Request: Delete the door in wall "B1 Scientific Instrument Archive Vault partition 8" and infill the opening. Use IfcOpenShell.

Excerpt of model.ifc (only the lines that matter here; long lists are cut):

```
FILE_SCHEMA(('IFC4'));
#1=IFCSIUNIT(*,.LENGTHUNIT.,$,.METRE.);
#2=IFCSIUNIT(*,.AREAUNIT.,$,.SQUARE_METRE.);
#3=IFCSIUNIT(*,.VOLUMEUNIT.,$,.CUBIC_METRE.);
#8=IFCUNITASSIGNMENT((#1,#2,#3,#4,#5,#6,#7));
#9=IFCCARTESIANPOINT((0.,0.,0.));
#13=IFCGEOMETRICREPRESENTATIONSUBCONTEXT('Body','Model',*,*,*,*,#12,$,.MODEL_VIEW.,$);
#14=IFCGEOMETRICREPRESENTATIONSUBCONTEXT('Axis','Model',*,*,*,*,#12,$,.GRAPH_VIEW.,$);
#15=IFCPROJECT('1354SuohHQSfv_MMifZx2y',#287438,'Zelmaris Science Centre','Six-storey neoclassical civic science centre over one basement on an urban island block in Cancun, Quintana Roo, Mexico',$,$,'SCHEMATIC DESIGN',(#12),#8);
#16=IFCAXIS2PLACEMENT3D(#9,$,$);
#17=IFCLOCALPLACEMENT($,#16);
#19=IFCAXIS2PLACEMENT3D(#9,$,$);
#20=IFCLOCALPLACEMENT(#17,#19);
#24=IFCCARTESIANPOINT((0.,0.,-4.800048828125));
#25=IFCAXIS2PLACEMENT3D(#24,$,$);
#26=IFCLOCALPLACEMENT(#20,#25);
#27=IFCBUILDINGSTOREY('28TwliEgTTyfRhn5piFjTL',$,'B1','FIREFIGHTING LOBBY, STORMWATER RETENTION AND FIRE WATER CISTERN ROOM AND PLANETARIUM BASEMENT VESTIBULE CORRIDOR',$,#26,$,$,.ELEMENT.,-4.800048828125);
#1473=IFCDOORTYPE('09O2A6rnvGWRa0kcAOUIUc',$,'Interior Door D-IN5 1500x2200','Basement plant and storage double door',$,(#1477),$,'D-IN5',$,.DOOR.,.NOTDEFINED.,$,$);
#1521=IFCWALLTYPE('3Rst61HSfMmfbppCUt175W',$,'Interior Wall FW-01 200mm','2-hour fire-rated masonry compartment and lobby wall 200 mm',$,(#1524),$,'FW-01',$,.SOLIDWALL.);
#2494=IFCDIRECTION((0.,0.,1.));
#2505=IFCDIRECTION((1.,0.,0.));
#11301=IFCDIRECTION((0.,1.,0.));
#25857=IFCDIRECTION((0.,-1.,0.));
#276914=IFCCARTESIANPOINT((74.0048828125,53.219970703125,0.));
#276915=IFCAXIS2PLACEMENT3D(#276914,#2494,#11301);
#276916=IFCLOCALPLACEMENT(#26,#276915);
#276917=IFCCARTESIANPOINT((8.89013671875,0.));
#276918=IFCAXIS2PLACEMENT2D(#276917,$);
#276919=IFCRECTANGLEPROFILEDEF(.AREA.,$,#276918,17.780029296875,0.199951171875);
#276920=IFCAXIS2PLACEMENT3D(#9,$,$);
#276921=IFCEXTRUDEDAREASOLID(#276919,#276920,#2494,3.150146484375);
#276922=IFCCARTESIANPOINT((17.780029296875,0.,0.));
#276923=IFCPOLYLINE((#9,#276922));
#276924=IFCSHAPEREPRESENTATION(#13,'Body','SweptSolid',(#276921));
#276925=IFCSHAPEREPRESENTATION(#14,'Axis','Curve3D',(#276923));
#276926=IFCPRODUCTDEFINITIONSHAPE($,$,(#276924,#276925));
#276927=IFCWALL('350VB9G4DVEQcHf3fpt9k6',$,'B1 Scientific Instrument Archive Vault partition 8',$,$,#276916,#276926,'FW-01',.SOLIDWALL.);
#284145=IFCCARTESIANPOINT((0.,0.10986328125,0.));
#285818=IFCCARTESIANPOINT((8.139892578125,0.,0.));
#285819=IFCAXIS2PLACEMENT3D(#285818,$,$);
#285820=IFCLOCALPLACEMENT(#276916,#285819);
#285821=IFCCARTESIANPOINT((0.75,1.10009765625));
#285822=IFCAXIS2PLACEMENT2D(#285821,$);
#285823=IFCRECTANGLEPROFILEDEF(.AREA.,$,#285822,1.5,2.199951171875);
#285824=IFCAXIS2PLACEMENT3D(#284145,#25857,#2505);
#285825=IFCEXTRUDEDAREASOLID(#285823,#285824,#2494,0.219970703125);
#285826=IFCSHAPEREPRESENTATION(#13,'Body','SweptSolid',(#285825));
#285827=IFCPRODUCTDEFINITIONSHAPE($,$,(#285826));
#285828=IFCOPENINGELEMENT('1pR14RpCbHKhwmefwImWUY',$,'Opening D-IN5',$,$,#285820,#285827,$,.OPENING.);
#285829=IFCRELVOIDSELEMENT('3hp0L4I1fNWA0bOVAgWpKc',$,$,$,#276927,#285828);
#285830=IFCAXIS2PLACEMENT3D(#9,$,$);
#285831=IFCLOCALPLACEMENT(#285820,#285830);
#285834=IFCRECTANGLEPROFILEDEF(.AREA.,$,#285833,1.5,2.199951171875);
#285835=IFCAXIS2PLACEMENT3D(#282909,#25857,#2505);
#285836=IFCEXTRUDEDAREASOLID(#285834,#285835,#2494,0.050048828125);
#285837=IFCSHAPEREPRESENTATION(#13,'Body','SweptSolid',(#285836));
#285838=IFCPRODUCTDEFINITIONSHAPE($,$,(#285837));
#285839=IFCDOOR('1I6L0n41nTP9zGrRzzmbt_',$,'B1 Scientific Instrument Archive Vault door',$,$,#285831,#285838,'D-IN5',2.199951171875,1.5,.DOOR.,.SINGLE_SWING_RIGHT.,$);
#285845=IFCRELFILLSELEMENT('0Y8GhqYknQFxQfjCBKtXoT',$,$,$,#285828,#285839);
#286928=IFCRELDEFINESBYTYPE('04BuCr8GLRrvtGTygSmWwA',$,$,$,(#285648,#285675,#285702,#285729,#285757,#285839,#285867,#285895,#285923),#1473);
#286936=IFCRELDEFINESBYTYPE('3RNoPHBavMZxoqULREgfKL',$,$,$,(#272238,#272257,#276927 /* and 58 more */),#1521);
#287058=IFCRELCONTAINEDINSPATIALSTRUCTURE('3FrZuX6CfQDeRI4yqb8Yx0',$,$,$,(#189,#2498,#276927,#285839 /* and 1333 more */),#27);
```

```python
import ifcopenshell
import ifcopenshell.api.feature
import ifcopenshell.api.root
import ifcopenshell.geom
import ifcopenshell.util.shape

model = ifcopenshell.open("model.ifc")
settings = ifcopenshell.geom.settings()


def volume(element):
    """Net volume in cubic metres, openings subtracted."""
    shape = ifcopenshell.geom.create_shape(settings, element)
    return ifcopenshell.util.shape.get_volume(shape.geometry)


door = model.by_guid("1I6L0n41nTP9zGrRzzmbt_")
opening = door.FillsVoids[0].RelatingOpeningElement
wall = opening.VoidsElements[0].RelatingBuildingElement
before = volume(wall)

ifcopenshell.api.root.remove_product(model, product=door)
ifcopenshell.api.feature.remove_feature(model, feature=opening)

after = volume(wall)

print(f"wall volume {before:.3f} -> {after:.3f} m3")

model.write("model_v2.ifc")
```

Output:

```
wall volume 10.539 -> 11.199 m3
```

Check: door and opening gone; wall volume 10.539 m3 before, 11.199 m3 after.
